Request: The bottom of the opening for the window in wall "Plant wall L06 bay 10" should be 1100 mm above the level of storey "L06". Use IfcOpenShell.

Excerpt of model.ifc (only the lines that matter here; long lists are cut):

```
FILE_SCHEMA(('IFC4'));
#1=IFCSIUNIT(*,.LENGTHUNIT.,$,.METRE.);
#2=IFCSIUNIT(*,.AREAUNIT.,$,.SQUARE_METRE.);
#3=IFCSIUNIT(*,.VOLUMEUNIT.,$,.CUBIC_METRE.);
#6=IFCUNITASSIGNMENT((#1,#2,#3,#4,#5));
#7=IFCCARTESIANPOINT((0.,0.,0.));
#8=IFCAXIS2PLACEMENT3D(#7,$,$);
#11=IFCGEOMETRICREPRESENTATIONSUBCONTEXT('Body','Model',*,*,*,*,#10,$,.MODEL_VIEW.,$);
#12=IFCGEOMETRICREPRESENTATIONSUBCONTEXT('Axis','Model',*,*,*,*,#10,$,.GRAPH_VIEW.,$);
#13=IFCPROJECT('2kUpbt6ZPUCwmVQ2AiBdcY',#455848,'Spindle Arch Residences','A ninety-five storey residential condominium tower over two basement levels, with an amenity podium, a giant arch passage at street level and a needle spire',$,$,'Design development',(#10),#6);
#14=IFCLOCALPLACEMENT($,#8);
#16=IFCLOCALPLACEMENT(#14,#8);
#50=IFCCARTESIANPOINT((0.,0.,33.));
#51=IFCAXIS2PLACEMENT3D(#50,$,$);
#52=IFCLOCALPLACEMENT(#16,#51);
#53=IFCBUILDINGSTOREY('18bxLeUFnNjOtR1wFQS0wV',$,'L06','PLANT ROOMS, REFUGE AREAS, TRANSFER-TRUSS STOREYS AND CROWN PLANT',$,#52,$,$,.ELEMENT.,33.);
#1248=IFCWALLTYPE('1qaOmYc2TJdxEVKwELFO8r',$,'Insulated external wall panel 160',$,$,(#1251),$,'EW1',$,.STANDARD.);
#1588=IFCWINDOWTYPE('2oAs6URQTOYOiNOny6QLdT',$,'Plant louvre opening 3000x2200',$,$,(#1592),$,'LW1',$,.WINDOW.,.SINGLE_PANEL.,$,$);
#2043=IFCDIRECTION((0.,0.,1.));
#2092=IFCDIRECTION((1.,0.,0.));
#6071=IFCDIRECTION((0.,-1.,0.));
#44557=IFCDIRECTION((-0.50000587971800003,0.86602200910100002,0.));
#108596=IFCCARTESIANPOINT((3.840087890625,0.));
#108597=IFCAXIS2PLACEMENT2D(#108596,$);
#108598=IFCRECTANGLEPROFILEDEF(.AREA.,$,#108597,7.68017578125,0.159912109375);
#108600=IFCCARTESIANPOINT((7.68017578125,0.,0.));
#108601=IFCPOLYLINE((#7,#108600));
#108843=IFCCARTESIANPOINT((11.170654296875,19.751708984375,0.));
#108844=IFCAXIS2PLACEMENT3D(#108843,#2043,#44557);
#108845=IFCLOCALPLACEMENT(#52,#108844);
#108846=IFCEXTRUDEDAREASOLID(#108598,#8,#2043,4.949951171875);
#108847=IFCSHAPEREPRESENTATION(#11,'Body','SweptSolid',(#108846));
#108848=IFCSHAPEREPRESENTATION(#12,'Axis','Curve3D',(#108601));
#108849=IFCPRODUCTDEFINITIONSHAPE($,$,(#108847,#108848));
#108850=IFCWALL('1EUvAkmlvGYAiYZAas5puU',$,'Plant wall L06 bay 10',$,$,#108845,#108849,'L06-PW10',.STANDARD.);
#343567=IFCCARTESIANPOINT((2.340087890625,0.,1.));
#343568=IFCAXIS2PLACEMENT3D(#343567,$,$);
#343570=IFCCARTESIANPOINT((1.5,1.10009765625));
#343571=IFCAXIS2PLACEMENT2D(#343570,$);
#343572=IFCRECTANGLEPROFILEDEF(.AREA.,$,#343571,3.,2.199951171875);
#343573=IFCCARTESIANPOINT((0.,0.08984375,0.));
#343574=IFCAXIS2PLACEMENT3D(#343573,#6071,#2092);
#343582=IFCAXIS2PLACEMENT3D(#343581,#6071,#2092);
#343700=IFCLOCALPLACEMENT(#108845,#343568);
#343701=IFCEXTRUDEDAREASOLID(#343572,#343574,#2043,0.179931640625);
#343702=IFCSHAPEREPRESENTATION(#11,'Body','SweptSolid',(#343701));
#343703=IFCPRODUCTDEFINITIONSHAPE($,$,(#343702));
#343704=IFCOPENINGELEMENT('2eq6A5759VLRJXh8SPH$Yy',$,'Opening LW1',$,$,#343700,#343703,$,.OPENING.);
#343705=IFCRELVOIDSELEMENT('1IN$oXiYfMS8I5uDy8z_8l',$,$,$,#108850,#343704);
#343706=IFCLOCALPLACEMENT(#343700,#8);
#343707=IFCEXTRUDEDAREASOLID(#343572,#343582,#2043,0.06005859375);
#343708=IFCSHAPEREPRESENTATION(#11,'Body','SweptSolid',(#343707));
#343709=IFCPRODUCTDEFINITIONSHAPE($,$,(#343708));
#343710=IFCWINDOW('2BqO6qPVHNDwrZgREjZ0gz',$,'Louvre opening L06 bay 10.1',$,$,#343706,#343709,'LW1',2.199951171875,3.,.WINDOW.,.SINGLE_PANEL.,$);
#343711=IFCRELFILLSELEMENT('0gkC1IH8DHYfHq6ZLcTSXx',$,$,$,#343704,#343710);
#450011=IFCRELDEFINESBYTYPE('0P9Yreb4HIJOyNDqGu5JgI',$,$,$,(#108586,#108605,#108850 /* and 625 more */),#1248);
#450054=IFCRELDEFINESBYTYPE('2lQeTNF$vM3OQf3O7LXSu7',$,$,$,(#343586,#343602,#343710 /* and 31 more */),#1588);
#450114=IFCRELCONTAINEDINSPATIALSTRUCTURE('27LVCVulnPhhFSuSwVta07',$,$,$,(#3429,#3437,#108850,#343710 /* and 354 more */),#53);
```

```python
import numpy as np
import ifcopenshell
import ifcopenshell.api.geometry
import ifcopenshell.geom
import ifcopenshell.util.element
import ifcopenshell.util.placement
import ifcopenshell.util.shape
import ifcopenshell.util.unit

model = ifcopenshell.open("model.ifc")
unit_scale = ifcopenshell.util.unit.calculate_unit_scale(model)

window = model.by_guid("2BqO6qPVHNDwrZgREjZ0gz")
opening = window.FillsVoids[0].RelatingOpeningElement
storey = ifcopenshell.util.element.get_container(window, ifc_class="IfcBuildingStorey")
level = ifcopenshell.util.placement.get_local_placement(storey.ObjectPlacement)[2, 3]

# The opening's origin need not be at the sill, so measure its lowest point.
shape = ifcopenshell.geom.create_shape(ifcopenshell.geom.settings(), opening)
bottom = ifcopenshell.util.shape.get_shape_bottom_elevation(shape, shape.geometry) / unit_scale
dz = level + 1.1 / unit_scale - bottom

shift = np.array([0.0, 0.0, dz])
# The window is placed relative to its opening, so it follows when the opening moves.
matrix = ifcopenshell.util.placement.get_local_placement(opening.ObjectPlacement)
matrix[:3, 3] += shift
ifcopenshell.api.geometry.edit_object_placement(
    model, product=opening, matrix=matrix, is_si=False, should_transform_children=True
)

print(f"moved by {dz * unit_scale:+.3f} m")

model.write("model-out.ifc")
```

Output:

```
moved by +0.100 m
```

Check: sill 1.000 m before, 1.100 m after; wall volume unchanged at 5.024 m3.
